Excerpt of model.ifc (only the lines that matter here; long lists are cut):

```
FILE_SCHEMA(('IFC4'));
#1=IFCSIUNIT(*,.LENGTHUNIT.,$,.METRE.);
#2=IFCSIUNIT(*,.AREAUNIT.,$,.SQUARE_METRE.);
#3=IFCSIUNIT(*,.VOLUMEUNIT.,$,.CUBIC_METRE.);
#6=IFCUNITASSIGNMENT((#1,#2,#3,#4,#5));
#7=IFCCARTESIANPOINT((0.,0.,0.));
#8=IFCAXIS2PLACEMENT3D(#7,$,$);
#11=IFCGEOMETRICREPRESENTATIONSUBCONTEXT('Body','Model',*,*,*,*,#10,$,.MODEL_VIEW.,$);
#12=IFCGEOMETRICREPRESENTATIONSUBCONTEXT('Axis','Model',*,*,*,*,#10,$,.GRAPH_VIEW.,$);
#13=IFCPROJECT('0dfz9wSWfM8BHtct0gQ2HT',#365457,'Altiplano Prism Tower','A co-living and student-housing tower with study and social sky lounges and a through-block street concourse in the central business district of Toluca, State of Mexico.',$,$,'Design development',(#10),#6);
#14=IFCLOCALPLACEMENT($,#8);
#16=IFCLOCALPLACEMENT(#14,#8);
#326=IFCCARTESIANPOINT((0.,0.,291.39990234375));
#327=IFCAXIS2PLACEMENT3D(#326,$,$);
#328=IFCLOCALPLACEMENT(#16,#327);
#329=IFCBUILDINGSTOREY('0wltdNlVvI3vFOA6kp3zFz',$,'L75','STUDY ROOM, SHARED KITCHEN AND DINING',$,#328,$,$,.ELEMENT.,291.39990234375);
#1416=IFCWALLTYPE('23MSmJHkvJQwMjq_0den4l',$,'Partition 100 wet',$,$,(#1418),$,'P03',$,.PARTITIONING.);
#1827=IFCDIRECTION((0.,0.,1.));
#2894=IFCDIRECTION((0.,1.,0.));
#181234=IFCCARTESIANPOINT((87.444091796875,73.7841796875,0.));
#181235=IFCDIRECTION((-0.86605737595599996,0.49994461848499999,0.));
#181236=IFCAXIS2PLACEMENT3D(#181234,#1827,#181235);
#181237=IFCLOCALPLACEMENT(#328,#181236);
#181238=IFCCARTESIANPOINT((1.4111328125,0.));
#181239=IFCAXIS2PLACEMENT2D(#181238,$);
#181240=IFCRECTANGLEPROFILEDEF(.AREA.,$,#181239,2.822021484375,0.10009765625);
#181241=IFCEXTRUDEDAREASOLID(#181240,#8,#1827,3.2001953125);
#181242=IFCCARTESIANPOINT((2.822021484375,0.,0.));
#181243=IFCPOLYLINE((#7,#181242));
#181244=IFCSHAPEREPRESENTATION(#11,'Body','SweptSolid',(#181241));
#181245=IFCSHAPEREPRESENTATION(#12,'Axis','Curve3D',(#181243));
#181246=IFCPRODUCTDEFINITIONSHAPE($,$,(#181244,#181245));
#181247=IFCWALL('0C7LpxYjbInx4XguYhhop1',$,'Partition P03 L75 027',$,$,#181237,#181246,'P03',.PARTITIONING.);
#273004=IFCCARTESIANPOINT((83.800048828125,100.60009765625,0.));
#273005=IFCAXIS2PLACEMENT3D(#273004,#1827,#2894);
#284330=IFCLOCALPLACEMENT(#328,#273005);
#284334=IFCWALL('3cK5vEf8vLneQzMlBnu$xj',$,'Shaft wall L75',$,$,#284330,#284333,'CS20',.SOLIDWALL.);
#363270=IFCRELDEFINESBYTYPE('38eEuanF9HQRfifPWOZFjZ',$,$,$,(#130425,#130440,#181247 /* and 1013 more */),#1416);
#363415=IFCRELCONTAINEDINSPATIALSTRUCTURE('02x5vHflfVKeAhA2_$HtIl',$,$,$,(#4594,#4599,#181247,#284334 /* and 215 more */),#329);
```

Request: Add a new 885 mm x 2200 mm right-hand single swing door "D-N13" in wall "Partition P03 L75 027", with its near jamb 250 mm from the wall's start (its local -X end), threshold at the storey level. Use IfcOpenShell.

```python
import numpy as np
import ifcopenshell
import ifcopenshell.api.feature
import ifcopenshell.api.geometry
import ifcopenshell.api.root
import ifcopenshell.api.spatial
import ifcopenshell.geom
import ifcopenshell.util.element
import ifcopenshell.util.placement
import ifcopenshell.util.representation
import ifcopenshell.util.shape
import ifcopenshell.util.unit

model = ifcopenshell.open("model.ifc")
unit_scale = ifcopenshell.util.unit.calculate_unit_scale(model)
settings = ifcopenshell.geom.settings()


def volume(element):
    """Net volume in cubic metres, openings subtracted."""
    shape = ifcopenshell.geom.create_shape(settings, element)
    return ifcopenshell.util.shape.get_volume(shape.geometry)


wall = model.by_id(181247)
storey = ifcopenshell.util.element.get_container(wall, ifc_class="IfcBuildingStorey")
context = ifcopenshell.util.representation.get_context(model, "Model", "Body", "MODEL_VIEW")
before = volume(wall)

width, height, from_end, sill = 0.885, 2.2, 0.25, 0.0  # metres

# The wall runs along its own X axis, and the end named is its -X end.
wall_shape = ifcopenshell.geom.create_shape(settings, wall)
x, y, z = ifcopenshell.util.shape.get_vertices(wall_shape.geometry).T
start = x.min() + from_end
face, thickness = float(y.min()), float(y.max() - y.min())
wall_matrix = ifcopenshell.util.placement.get_local_placement(wall.ObjectPlacement)
level = ifcopenshell.util.placement.get_local_placement(storey.ObjectPlacement)[2, 3]


def in_wall(x, y):
    """Placement at x, y metres in the wall's axes, at sill height."""
    matrix = wall_matrix.copy()
    matrix[:, 3] = wall_matrix @ np.array([x / unit_scale, y / unit_scale, 0.0, 1.0])
    matrix[2, 3] = level + sill / unit_scale
    return matrix


# Opening: a box that overshoots both wall faces by 50 mm.
opening = ifcopenshell.api.root.create_entity(model, ifc_class="IfcOpeningElement", predefined_type="OPENING")
box = ifcopenshell.api.geometry.add_wall_representation(
    model, context=context, length=width, height=height, thickness=thickness + 0.1
)
ifcopenshell.api.geometry.assign_representation(model, product=opening, representation=box)
ifcopenshell.api.geometry.edit_object_placement(model, product=opening, matrix=in_wall(start, face - 0.05), is_si=False)
ifcopenshell.api.feature.add_feature(model, feature=opening, element=wall)

door = ifcopenshell.api.root.create_entity(model, ifc_class="IfcDoor", name="D-N13", predefined_type="DOOR")
door.OverallWidth, door.OverallHeight = width / unit_scale, height / unit_scale
door.OperationType = "SINGLE_SWING_RIGHT"
body = ifcopenshell.api.geometry.add_door_representation(
    model,
    context=context,
    overall_width=door.OverallWidth,
    overall_height=door.OverallHeight,
    operation_type="SINGLE_SWING_RIGHT",
    lining_properties={"LiningDepth": thickness / unit_scale, "ThresholdDepth": thickness / unit_scale},
)
ifcopenshell.api.geometry.assign_representation(model, product=door, representation=body)
ifcopenshell.api.spatial.assign_container(model, products=[door], relating_structure=storey)
ifcopenshell.api.feature.add_filling(model, opening=opening, element=door)

# The lining spans the wall, so the door starts at the wall face.
ifcopenshell.api.geometry.edit_object_placement(model, product=door, matrix=in_wall(start, face), is_si=False)

after = volume(wall)

print(f"wall volume {before:.3f} -> {after:.3f} m3")

model.write("model_edited.ifc")
```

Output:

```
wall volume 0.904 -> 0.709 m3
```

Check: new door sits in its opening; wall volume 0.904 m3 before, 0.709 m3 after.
